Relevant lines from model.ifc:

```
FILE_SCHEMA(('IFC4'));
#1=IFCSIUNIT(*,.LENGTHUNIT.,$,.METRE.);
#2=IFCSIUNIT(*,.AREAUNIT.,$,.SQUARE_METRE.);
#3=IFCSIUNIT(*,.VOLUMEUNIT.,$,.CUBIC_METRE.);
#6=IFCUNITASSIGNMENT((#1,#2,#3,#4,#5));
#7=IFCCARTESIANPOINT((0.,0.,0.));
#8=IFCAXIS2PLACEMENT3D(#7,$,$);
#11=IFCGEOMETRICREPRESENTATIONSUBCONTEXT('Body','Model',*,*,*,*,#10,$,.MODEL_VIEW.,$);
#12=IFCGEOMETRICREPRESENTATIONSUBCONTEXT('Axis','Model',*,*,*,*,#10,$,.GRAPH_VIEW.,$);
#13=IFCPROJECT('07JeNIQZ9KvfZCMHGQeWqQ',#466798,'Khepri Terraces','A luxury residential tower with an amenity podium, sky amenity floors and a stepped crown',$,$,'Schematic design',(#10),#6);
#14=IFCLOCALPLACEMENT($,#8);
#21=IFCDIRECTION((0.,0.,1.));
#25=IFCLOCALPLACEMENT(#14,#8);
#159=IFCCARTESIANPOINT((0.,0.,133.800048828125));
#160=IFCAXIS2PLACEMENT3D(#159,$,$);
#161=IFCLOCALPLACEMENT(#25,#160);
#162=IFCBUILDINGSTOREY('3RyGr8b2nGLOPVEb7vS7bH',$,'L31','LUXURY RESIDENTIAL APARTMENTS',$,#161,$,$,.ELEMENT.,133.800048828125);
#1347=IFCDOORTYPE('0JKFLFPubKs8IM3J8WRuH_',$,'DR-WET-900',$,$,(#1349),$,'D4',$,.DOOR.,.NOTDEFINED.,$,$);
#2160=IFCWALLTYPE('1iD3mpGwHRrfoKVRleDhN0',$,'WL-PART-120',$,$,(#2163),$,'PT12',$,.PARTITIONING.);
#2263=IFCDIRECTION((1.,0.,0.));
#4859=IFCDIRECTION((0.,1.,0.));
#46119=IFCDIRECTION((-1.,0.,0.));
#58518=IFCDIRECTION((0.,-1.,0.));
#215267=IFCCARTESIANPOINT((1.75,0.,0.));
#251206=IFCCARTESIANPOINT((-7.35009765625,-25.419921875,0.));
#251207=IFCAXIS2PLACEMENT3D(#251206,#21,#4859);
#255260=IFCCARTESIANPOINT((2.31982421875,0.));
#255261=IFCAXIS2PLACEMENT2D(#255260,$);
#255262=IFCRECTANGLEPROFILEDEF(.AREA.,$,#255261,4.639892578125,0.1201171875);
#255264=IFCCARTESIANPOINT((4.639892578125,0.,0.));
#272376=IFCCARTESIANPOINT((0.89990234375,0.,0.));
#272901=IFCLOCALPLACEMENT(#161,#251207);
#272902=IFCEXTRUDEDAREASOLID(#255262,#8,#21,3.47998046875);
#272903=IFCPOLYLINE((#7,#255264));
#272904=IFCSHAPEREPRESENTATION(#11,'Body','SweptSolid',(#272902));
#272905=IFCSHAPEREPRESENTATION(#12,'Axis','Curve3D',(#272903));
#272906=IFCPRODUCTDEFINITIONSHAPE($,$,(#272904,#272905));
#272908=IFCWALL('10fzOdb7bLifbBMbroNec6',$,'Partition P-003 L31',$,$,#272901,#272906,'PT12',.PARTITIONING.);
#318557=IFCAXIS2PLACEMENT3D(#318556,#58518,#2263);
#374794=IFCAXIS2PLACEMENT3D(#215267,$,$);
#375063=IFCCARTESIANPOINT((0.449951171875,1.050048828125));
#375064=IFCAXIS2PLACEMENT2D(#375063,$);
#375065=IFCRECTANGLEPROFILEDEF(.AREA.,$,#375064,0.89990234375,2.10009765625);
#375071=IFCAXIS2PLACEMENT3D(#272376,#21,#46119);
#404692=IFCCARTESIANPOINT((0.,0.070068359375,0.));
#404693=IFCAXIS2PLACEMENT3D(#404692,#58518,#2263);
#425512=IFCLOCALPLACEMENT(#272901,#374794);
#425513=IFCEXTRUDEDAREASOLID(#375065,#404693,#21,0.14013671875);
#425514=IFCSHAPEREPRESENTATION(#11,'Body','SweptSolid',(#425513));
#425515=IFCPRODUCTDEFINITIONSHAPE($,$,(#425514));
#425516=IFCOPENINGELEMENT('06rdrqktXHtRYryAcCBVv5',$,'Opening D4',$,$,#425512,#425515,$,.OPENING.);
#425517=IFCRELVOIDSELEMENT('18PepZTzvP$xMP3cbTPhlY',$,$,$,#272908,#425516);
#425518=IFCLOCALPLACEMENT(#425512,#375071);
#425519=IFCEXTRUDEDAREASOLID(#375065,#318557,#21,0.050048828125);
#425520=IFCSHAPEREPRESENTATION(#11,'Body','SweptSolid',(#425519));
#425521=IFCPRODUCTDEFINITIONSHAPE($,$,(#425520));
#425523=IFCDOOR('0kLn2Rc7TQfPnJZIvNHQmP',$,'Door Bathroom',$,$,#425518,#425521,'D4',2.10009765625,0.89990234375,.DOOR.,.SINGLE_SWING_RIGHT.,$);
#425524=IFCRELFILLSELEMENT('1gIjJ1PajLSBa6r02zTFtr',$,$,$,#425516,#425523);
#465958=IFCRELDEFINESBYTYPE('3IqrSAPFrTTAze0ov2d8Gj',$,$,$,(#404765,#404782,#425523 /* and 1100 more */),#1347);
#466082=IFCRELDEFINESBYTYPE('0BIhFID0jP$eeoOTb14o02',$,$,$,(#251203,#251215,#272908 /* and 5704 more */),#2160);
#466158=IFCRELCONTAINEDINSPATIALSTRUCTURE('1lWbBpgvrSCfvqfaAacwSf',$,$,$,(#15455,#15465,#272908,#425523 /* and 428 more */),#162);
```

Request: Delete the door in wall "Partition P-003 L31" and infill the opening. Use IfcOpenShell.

```python
import ifcopenshell
import ifcopenshell.api.feature
import ifcopenshell.api.root
import ifcopenshell.geom
import ifcopenshell.util.shape

model = ifcopenshell.open("model.ifc")
settings = ifcopenshell.geom.settings()


def volume(element):
    """Net volume in cubic metres, openings subtracted."""
    shape = ifcopenshell.geom.create_shape(settings, element)
    return ifcopenshell.util.shape.get_volume(shape.geometry)


door = model.by_guid("0kLn2Rc7TQfPnJZIvNHQmP")
opening = door.FillsVoids[0].RelatingOpeningElement
wall = opening.VoidsElements[0].RelatingBuildingElement
before = volume(wall)

ifcopenshell.api.root.remove_product(model, product=door)
ifcopenshell.api.feature.remove_feature(model, feature=opening)

after = volume(wall)

print(f"wall volume {before:.3f} -> {after:.3f} m3")

model.write("model_rev.ifc")
```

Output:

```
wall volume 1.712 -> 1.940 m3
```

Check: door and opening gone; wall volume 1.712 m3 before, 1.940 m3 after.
